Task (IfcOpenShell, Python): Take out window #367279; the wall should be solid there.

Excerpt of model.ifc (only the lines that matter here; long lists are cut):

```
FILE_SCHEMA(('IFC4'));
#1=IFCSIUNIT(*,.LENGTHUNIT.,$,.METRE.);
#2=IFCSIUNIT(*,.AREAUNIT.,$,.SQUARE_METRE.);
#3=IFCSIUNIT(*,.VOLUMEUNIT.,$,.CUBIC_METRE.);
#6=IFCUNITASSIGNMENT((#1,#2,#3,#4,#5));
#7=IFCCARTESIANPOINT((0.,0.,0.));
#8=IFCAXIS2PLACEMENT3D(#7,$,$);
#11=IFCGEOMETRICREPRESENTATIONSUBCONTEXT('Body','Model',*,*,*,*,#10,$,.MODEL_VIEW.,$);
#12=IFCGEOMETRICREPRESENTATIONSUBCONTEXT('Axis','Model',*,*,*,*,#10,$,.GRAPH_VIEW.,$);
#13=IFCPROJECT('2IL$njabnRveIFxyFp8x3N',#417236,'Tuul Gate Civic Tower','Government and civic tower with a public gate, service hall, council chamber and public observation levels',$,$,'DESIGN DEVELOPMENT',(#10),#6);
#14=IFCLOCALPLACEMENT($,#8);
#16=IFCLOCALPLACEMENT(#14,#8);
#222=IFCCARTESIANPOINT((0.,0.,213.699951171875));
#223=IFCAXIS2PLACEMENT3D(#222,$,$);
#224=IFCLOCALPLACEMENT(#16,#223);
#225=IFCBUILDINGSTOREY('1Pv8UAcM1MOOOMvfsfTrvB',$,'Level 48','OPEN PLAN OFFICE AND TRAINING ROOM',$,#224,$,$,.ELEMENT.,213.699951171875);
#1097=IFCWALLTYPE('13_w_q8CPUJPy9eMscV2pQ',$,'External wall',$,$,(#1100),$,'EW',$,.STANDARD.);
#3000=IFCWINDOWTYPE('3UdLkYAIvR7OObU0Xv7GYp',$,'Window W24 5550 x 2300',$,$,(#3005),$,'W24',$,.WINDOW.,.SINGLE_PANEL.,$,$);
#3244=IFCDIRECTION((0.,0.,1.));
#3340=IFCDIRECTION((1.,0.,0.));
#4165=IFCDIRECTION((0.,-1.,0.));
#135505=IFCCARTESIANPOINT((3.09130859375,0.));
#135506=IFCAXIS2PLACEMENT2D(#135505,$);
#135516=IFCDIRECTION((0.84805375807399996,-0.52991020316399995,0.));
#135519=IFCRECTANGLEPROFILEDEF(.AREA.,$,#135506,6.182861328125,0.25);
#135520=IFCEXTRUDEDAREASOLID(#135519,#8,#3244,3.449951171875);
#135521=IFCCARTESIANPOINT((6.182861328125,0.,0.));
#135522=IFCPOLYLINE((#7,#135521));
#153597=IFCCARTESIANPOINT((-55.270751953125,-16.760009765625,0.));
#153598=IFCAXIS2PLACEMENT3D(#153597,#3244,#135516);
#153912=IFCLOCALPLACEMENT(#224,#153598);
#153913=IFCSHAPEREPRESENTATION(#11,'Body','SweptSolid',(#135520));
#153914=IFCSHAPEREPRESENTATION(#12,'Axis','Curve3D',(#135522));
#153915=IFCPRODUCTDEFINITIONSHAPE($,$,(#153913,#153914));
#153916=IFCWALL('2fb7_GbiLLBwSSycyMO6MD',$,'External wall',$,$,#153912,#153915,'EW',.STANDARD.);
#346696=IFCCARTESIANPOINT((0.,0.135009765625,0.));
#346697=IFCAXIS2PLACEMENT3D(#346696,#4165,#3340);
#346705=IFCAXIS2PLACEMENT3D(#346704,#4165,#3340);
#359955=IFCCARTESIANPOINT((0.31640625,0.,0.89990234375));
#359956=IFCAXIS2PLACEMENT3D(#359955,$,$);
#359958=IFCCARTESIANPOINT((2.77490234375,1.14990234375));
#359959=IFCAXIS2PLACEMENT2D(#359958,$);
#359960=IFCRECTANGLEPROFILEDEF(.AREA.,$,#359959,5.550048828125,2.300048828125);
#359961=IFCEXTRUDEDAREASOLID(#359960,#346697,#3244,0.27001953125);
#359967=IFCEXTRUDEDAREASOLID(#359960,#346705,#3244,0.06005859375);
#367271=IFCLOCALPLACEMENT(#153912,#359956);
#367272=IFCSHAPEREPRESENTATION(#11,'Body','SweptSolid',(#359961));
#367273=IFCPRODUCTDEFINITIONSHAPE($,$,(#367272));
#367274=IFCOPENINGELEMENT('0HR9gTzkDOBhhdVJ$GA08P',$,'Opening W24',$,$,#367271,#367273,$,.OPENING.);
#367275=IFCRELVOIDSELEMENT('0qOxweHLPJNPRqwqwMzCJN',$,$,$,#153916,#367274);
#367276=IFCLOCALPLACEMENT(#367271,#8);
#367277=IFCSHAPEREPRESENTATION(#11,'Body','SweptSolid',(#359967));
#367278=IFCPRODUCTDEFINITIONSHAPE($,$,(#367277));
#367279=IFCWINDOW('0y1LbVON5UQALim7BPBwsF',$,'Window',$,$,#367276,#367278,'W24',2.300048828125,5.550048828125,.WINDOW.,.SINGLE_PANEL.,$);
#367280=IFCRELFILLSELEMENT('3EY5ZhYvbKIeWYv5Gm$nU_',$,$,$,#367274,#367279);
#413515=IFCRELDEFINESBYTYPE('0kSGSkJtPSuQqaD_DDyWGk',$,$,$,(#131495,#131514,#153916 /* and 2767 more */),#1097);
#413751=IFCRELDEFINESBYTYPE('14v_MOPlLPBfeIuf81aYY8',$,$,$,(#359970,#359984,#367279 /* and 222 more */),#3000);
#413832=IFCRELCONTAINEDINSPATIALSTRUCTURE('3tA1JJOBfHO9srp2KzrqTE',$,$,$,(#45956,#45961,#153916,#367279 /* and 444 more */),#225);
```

```python
import ifcopenshell
import ifcopenshell.api.feature
import ifcopenshell.api.root
import ifcopenshell.geom
import ifcopenshell.util.shape

model = ifcopenshell.open("model.ifc")
settings = ifcopenshell.geom.settings()


def volume(element):
    """Net volume in cubic metres, openings subtracted."""
    shape = ifcopenshell.geom.create_shape(settings, element)
    return ifcopenshell.util.shape.get_volume(shape.geometry)


window = model.by_guid("0y1LbVON5UQALim7BPBwsF")
opening = window.FillsVoids[0].RelatingOpeningElement
wall = opening.VoidsElements[0].RelatingBuildingElement
before = volume(wall)

ifcopenshell.api.root.remove_product(model, product=window)
ifcopenshell.api.feature.remove_feature(model, feature=opening)

after = volume(wall)

print(f"wall volume {before:.3f} -> {after:.3f} m3")

model.write("model-out.ifc")
```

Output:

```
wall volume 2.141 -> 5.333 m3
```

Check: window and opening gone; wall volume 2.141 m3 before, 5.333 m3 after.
